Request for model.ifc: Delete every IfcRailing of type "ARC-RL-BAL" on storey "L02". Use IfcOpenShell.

First a look at what the model holds.

```python
import ifcopenshell
import ifcopenshell.util.element

model = ifcopenshell.open("model.ifc")
print(model.schema)
storey = next(s for s in model.by_type("IfcBuildingStorey") if s.Name == "L02")
railings = [e for e in ifcopenshell.util.element.get_decomposition(storey) if e.is_a("IfcRailing")]
seen = {}
for e in railings:
    element_type = ifcopenshell.util.element.get_type(e)
    name = element_type.Name if element_type not in (None, e) else None
    seen[name] = seen.get(name, 0) + 1
for name, count in sorted(seen.items(), key=str):
    print(count, "x", name)
```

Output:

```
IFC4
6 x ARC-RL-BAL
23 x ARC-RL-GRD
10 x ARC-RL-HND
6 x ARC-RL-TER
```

```python
import ifcopenshell
import ifcopenshell.api.root
import ifcopenshell.util.element

model = ifcopenshell.open("model.ifc")

storey = next(s for s in model.by_type("IfcBuildingStorey") if s.Name == "L02")
railings = [e for e in ifcopenshell.util.element.get_decomposition(storey) if e.is_a("IfcRailing")]
targets = [e for e in railings if (t := ifcopenshell.util.element.get_type(e)) not in (None, e) and t.Name == "ARC-RL-BAL"]

for e in targets:
    ifcopenshell.api.root.remove_product(model, product=e)
print(len(targets), "removed")

model.write("model-out.ifc")
```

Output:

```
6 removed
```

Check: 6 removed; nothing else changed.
